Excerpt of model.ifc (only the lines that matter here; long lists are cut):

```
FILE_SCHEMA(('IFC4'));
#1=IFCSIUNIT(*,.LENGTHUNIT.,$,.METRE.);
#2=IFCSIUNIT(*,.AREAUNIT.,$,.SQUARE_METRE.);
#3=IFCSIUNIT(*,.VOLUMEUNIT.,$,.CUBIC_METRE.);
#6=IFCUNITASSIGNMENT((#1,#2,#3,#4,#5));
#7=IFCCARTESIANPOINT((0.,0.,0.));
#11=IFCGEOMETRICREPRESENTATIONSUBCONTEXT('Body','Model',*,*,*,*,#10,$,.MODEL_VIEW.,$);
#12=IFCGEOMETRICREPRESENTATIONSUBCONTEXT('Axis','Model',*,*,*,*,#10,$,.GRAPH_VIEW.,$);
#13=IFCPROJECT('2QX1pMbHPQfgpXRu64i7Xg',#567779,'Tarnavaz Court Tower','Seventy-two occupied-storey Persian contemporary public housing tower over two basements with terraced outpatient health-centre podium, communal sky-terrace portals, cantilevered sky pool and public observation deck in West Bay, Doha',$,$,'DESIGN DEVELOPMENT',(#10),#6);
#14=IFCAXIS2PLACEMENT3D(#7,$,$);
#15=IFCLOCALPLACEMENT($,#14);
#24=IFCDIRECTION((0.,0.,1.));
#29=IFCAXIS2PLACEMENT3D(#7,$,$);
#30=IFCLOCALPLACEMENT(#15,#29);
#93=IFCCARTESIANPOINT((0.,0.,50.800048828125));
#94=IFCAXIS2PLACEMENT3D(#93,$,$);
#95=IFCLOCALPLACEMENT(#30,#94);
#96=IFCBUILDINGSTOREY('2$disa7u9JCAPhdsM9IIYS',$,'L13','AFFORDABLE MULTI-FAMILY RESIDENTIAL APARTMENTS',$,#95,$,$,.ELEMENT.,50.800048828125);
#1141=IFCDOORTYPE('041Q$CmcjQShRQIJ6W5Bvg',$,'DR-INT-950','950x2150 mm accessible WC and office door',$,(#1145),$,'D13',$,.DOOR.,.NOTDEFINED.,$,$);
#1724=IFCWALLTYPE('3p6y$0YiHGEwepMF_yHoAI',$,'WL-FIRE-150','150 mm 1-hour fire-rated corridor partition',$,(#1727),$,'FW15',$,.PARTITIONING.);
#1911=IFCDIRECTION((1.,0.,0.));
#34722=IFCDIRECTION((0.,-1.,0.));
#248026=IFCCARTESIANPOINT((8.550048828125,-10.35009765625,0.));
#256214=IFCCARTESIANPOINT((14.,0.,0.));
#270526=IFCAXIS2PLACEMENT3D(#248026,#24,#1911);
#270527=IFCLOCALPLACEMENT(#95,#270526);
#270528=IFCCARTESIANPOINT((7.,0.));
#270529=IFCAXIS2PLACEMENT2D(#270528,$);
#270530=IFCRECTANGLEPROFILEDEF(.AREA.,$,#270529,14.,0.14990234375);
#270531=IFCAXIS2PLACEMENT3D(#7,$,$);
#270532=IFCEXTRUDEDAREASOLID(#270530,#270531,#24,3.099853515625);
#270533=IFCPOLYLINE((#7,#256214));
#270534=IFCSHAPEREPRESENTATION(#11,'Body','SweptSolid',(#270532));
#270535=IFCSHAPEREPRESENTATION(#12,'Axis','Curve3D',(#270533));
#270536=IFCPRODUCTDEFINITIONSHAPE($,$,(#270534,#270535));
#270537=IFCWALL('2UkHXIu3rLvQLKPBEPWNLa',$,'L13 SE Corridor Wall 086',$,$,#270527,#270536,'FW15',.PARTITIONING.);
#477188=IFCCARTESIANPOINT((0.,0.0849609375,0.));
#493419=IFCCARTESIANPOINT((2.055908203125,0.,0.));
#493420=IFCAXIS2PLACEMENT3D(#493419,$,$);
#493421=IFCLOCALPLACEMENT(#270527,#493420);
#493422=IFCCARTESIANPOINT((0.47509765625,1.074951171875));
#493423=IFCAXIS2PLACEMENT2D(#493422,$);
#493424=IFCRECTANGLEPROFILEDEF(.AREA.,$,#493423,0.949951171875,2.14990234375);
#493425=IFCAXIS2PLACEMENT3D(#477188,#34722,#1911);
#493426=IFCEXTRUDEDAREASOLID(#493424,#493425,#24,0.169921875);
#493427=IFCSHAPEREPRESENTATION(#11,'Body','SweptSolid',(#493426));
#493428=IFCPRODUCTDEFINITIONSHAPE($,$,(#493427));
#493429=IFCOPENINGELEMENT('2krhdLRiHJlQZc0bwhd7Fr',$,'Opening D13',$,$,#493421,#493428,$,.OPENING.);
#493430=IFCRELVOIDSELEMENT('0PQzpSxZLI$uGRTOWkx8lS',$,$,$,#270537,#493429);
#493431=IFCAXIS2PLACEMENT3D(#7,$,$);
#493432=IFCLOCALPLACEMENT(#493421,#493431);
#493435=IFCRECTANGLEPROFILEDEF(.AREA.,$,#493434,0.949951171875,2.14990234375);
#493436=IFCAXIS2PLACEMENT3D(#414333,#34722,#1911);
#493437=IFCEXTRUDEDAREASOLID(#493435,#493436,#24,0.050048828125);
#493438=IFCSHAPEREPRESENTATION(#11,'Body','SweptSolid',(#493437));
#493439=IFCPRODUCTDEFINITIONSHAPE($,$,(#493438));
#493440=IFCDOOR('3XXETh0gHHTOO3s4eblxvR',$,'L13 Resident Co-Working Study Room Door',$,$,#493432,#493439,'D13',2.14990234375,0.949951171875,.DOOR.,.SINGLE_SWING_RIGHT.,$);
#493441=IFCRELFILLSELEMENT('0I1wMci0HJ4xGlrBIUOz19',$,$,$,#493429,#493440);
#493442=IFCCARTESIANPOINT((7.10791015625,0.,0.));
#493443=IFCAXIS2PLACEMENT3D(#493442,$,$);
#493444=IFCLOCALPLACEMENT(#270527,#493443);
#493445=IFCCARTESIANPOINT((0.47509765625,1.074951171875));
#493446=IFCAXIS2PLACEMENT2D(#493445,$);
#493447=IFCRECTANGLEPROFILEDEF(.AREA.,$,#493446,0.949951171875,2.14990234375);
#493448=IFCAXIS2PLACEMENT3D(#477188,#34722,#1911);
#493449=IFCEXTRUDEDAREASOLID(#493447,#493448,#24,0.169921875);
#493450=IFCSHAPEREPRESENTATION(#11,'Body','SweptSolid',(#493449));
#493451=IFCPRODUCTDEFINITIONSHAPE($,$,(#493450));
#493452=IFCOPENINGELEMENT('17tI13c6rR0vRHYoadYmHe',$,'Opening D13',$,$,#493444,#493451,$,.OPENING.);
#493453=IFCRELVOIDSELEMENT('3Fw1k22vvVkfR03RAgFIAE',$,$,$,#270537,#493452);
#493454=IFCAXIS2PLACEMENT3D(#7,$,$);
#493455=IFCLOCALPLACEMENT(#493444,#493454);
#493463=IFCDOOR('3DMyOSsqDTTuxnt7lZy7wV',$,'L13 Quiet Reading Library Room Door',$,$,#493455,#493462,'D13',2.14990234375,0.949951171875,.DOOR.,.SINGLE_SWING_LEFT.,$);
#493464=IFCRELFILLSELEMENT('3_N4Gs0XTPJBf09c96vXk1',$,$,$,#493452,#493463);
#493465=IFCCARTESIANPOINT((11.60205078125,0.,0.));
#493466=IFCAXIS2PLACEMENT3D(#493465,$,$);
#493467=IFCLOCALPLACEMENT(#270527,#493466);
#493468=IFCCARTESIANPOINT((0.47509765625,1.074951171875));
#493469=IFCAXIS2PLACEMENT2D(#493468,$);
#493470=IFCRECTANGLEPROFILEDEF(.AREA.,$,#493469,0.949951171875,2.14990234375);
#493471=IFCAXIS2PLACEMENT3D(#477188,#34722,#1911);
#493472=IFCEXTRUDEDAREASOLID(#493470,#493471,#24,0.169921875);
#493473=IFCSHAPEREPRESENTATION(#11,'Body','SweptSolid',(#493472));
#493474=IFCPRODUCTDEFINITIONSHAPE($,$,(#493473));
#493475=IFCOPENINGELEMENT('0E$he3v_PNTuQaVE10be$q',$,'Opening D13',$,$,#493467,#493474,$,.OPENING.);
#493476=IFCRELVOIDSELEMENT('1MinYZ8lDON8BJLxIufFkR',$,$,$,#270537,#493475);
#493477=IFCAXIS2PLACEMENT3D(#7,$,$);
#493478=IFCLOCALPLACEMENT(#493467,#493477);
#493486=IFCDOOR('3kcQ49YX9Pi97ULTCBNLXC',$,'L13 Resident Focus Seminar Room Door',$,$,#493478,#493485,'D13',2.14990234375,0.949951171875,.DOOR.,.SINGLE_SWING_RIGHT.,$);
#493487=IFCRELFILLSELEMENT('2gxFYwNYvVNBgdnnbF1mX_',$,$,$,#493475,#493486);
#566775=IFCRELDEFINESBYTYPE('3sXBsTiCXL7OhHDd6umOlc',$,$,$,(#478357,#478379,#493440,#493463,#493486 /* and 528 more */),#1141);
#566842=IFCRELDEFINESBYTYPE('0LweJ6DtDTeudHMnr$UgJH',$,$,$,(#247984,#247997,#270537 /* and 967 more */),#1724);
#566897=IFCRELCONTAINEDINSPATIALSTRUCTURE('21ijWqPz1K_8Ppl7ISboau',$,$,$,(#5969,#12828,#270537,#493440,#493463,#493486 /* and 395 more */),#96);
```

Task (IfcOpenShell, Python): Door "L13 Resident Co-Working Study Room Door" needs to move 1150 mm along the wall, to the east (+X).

```python
import ifcopenshell
import ifcopenshell.api.geometry
import ifcopenshell.util.placement

model = ifcopenshell.open("model.ifc")

door = model.by_id(493440)
opening = door.FillsVoids[0].RelatingOpeningElement
wall = opening.VoidsElements[0].RelatingBuildingElement

wall_matrix = ifcopenshell.util.placement.get_local_placement(wall.ObjectPlacement)
shift = wall_matrix[:3, 0] * 1.15
before = ifcopenshell.util.placement.get_local_placement(door.ObjectPlacement)[:3, 3].copy()

# The door is placed relative to its opening, so it follows when the opening moves.
matrix = ifcopenshell.util.placement.get_local_placement(opening.ObjectPlacement)
matrix[:3, 3] += shift
ifcopenshell.api.geometry.edit_object_placement(
    model, product=opening, matrix=matrix, is_si=False, should_transform_children=True
)

after = ifcopenshell.util.placement.get_local_placement(door.ObjectPlacement)[:3, 3]
print("door moved by", (after - before).round(3) + 0.0)

model.write("model_edited.ifc")
```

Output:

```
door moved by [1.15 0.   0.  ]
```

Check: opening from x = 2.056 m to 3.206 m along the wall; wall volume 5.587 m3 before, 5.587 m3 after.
